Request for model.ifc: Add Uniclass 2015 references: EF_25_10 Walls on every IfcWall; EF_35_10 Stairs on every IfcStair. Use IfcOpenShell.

First a look at what the model holds.

```python
import ifcopenshell

model = ifcopenshell.open("model.ifc")
print(model.schema)
print("classifications:", [c.Name for c in model.by_type("IfcClassification")])
for ifc_class in ("IfcDoor", "IfcRoof", "IfcStair", "IfcWall", "IfcWindow"):
    print(ifc_class, len(model.by_type(ifc_class)))
```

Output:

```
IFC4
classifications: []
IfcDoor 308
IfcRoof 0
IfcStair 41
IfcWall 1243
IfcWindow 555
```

```python
import ifcopenshell
import ifcopenshell.api.classification

model = ifcopenshell.open("model.ifc")

system = ifcopenshell.api.classification.add_classification(model, classification="Uniclass 2015")

codes = {
    "IfcWall": ("EF_25_10", "Walls"),
    "IfcStair": ("EF_35_10", "Stairs"),
}
for ifc_class, (code, name) in codes.items():
    products = model.by_type(ifc_class)
    ifcopenshell.api.classification.add_reference(
        model, products=products, classification=system, identification=code, name=name
    )
    print(code, len(products))

model.write("model_edited.ifc")
```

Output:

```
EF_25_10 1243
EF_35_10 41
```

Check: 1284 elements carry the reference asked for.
